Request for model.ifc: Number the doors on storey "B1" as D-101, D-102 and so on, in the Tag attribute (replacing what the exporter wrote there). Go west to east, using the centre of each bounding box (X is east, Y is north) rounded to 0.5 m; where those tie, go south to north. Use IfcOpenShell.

First a look at what the model holds.

```python
import ifcopenshell
import ifcopenshell.util.element
import ifcopenshell.util.placement

model = ifcopenshell.open("model.ifc")
print(model.schema)
storey = next(s for s in model.by_type("IfcBuildingStorey") if s.Name == "B1")
doors = [e for e in ifcopenshell.util.element.get_decomposition(storey) if e.is_a("IfcDoor")]
for e in sorted(doors, key=lambda e: e.id()):
    origin = ifcopenshell.util.placement.get_local_placement(e.ObjectPlacement)[:3, 3]
    print(e.id(), e.Tag, e.Name, origin.round(2) + 0.0, sep=" | ")
```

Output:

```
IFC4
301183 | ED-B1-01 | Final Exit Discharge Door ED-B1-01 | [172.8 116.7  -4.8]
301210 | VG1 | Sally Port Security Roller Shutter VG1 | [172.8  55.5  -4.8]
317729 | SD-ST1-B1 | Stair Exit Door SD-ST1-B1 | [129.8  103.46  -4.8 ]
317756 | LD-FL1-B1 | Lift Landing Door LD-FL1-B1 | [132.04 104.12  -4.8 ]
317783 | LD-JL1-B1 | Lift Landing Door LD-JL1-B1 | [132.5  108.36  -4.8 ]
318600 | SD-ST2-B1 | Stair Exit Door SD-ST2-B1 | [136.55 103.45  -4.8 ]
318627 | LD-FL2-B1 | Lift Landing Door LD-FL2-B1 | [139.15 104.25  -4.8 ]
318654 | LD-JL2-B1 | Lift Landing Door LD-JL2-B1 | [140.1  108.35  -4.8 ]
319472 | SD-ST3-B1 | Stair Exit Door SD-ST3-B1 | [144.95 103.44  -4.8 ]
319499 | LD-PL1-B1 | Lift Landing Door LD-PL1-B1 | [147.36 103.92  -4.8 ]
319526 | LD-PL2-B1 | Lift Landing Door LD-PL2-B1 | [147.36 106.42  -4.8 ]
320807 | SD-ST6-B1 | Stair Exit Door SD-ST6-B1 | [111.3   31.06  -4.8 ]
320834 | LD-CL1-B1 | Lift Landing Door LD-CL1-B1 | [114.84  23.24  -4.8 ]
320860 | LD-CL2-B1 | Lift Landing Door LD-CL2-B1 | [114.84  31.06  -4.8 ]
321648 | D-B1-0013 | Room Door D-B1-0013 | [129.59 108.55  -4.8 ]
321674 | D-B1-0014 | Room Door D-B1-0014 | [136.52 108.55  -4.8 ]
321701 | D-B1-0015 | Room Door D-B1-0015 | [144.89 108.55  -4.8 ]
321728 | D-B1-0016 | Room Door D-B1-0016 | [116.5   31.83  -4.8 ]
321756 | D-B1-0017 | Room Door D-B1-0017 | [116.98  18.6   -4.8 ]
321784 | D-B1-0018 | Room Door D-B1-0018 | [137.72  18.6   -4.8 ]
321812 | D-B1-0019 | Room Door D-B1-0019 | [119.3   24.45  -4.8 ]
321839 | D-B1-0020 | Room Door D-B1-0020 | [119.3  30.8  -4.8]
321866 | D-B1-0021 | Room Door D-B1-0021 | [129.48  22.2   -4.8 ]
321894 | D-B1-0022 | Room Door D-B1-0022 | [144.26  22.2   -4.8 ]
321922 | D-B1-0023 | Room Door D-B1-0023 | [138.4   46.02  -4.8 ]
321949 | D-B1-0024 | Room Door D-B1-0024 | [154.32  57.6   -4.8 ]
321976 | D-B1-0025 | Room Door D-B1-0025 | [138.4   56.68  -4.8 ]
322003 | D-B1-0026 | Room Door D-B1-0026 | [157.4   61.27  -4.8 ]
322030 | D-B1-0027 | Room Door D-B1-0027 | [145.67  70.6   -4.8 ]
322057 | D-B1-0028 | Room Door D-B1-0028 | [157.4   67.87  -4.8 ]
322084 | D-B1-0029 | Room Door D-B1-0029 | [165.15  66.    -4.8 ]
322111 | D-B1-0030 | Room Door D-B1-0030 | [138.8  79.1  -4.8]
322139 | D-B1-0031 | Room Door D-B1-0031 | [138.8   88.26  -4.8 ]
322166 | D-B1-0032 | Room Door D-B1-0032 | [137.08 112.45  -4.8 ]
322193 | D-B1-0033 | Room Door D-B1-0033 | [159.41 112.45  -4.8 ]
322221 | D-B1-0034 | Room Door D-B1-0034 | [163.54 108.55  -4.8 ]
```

```python
import ifcopenshell
import ifcopenshell.geom
import ifcopenshell.util.element
import ifcopenshell.util.shape

model = ifcopenshell.open("model.ifc")
settings = ifcopenshell.geom.settings()
settings.set("use-world-coords", True)


def centre(element):
    shape = ifcopenshell.geom.create_shape(settings, element)
    return ifcopenshell.util.shape.get_bbox_centroid(shape.geometry)


storey = next(s for s in model.by_type("IfcBuildingStorey") if s.Name == "B1")
doors = [e for e in ifcopenshell.util.element.get_decomposition(storey) if e.is_a("IfcDoor")]

# Insertion points can sit at a corner or the storey origin, so sort by the geometry (in metres).
centres = {e: centre(e) for e in doors}
doors.sort(key=lambda e: (round(centres[e][0] / 0.5), centres[e][1]))

for i, e in enumerate(doors, start=1):
    number = f"D-1{i:02d}"
    e.Tag = number
    print(e.id(), number)

model.write("model_v2.ifc")
```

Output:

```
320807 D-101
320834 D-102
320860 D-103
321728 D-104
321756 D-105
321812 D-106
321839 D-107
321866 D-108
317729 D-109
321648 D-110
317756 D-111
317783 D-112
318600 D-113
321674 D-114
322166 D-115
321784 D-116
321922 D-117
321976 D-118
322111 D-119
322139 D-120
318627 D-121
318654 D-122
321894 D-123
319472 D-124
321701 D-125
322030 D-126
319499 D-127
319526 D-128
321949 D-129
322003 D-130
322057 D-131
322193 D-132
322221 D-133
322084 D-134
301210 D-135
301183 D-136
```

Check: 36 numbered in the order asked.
